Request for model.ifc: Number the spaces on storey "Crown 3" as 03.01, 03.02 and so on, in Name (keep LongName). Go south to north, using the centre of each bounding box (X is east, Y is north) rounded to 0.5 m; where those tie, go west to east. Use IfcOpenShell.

First a look at what the model holds.

```python
import ifcopenshell
import ifcopenshell.util.element
import ifcopenshell.util.placement

model = ifcopenshell.open("model.ifc")
print(model.schema)
storey = next(s for s in model.by_type("IfcBuildingStorey") if s.Name == "Crown 3")
spaces = [e for e in ifcopenshell.util.element.get_decomposition(storey) if e.is_a("IfcSpace")]
for e in sorted(spaces, key=lambda e: e.id()):
    origin = ifcopenshell.util.placement.get_local_placement(e.ObjectPlacement)[:3, 3]
    print(e.id(), e.Name, e.LongName, origin.round(2) + 0.0, sep=" | ")
```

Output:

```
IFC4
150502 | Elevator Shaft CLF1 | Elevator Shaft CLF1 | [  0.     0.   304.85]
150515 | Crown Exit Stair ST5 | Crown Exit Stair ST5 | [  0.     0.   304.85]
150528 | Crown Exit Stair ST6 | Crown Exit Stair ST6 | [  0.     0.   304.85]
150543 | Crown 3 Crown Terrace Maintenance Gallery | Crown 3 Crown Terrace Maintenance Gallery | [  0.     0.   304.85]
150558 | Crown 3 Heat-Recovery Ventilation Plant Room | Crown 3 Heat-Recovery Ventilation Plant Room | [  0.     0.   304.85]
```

```python
import ifcopenshell
import ifcopenshell.geom
import ifcopenshell.util.element
import ifcopenshell.util.shape

model = ifcopenshell.open("model.ifc")
settings = ifcopenshell.geom.settings()
settings.set("use-world-coords", True)


def centre(element):
    shape = ifcopenshell.geom.create_shape(settings, element)
    return ifcopenshell.util.shape.get_bbox_centroid(shape.geometry)


storey = next(s for s in model.by_type("IfcBuildingStorey") if s.Name == "Crown 3")
spaces = [e for e in ifcopenshell.util.element.get_decomposition(storey) if e.is_a("IfcSpace")]

# Insertion points can sit at a corner or the storey origin, so sort by the geometry (in metres).
centres = {e: centre(e) for e in spaces}
spaces.sort(key=lambda e: (round(centres[e][1] / 0.5), centres[e][0]))

for i, e in enumerate(spaces, start=1):
    number = f"03.{i:02d}"
    e.Name = number
    print(e.id(), number)

model.write("model_rev.ifc")
```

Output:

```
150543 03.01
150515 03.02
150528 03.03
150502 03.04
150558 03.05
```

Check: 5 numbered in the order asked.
